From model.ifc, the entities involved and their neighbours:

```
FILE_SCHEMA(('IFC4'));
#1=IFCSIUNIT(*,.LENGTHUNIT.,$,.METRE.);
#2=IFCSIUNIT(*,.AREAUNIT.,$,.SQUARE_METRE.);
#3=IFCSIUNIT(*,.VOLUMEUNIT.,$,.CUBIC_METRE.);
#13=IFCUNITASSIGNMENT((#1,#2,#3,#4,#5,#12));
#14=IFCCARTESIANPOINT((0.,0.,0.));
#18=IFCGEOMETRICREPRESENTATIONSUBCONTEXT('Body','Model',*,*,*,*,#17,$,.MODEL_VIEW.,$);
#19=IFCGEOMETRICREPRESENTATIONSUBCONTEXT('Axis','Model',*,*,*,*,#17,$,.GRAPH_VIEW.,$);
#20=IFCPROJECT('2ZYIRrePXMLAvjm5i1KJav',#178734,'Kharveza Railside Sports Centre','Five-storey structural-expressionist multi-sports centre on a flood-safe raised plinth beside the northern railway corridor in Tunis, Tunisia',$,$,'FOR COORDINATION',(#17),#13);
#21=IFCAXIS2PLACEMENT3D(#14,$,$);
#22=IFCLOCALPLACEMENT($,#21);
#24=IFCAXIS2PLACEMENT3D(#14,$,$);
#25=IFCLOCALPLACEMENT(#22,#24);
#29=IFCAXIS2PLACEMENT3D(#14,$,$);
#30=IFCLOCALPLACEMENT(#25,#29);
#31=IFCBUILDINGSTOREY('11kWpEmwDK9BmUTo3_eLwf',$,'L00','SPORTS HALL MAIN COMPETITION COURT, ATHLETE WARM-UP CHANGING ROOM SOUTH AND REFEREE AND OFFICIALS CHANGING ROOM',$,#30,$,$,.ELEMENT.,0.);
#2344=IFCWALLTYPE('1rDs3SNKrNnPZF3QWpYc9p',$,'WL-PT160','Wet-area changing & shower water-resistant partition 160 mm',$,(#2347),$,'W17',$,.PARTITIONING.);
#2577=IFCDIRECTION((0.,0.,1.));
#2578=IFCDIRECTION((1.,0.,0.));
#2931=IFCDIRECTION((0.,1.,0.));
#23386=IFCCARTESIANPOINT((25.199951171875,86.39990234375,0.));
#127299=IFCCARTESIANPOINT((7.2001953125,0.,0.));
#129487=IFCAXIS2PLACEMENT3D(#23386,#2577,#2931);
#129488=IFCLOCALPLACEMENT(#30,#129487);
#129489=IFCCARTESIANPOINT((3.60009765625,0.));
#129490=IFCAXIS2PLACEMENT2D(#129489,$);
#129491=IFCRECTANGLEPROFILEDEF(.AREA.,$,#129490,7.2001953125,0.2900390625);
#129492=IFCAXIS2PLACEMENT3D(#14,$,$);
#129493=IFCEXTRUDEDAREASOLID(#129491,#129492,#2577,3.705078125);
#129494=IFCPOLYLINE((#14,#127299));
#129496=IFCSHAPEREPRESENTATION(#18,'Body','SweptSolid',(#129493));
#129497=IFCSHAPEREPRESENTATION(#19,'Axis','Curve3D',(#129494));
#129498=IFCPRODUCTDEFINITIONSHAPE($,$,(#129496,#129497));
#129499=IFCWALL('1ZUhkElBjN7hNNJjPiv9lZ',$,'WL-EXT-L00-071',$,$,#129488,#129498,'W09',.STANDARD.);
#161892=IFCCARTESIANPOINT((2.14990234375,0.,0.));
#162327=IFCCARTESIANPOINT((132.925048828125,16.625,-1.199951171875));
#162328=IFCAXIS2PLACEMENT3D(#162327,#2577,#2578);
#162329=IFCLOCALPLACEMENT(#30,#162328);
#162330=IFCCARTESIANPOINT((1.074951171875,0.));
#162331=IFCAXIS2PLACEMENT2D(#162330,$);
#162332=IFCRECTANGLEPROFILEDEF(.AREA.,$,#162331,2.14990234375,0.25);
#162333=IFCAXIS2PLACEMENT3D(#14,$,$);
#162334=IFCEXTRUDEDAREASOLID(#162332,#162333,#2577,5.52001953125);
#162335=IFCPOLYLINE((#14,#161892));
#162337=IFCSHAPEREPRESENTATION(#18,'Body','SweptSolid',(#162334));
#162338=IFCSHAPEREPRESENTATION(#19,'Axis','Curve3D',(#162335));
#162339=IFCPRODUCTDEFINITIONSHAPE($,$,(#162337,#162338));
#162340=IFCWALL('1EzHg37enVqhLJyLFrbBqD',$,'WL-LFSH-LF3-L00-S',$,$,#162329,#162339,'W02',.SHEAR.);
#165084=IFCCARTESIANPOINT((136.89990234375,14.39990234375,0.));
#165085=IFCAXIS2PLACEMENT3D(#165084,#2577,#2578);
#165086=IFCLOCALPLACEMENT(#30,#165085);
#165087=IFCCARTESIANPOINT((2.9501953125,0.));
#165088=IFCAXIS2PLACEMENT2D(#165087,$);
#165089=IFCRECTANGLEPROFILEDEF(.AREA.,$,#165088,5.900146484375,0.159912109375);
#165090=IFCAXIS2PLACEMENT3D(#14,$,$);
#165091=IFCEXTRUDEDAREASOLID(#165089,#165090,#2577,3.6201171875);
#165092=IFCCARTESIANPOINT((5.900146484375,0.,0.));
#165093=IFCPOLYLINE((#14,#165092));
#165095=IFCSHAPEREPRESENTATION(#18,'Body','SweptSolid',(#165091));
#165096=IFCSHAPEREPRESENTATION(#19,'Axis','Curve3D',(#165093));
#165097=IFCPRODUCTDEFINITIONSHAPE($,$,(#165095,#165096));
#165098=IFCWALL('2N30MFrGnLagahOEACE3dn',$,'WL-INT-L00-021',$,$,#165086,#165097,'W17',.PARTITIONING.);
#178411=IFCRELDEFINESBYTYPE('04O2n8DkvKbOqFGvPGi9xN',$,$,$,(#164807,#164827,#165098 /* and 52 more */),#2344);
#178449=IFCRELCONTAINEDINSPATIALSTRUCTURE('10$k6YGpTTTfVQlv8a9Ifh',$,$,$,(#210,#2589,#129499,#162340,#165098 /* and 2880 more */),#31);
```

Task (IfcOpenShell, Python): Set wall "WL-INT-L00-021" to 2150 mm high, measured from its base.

```python
import ifcopenshell
import ifcopenshell.geom
import ifcopenshell.util.representation
import ifcopenshell.util.shape

model = ifcopenshell.open("model.ifc")
settings = ifcopenshell.geom.settings()


def volume(element):
    """Net volume in cubic metres, openings subtracted."""
    shape = ifcopenshell.geom.create_shape(settings, element)
    return ifcopenshell.util.shape.get_volume(shape.geometry)


wall = model.by_guid("2N30MFrGnLagahOEACE3dn")
before = volume(wall)

body = ifcopenshell.util.representation.get_representation(wall, "Model", "Body")
solid = body.Items[0]
old_height = solid.Depth
solid.Depth = 2.15
after = volume(wall)

print(f"height {old_height:g} -> {solid.Depth:g}, volume {before:.3f} -> {after:.3f} m3")

model.write("model_updated.ifc")
```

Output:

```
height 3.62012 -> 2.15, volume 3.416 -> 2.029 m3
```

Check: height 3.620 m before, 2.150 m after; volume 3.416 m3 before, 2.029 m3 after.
